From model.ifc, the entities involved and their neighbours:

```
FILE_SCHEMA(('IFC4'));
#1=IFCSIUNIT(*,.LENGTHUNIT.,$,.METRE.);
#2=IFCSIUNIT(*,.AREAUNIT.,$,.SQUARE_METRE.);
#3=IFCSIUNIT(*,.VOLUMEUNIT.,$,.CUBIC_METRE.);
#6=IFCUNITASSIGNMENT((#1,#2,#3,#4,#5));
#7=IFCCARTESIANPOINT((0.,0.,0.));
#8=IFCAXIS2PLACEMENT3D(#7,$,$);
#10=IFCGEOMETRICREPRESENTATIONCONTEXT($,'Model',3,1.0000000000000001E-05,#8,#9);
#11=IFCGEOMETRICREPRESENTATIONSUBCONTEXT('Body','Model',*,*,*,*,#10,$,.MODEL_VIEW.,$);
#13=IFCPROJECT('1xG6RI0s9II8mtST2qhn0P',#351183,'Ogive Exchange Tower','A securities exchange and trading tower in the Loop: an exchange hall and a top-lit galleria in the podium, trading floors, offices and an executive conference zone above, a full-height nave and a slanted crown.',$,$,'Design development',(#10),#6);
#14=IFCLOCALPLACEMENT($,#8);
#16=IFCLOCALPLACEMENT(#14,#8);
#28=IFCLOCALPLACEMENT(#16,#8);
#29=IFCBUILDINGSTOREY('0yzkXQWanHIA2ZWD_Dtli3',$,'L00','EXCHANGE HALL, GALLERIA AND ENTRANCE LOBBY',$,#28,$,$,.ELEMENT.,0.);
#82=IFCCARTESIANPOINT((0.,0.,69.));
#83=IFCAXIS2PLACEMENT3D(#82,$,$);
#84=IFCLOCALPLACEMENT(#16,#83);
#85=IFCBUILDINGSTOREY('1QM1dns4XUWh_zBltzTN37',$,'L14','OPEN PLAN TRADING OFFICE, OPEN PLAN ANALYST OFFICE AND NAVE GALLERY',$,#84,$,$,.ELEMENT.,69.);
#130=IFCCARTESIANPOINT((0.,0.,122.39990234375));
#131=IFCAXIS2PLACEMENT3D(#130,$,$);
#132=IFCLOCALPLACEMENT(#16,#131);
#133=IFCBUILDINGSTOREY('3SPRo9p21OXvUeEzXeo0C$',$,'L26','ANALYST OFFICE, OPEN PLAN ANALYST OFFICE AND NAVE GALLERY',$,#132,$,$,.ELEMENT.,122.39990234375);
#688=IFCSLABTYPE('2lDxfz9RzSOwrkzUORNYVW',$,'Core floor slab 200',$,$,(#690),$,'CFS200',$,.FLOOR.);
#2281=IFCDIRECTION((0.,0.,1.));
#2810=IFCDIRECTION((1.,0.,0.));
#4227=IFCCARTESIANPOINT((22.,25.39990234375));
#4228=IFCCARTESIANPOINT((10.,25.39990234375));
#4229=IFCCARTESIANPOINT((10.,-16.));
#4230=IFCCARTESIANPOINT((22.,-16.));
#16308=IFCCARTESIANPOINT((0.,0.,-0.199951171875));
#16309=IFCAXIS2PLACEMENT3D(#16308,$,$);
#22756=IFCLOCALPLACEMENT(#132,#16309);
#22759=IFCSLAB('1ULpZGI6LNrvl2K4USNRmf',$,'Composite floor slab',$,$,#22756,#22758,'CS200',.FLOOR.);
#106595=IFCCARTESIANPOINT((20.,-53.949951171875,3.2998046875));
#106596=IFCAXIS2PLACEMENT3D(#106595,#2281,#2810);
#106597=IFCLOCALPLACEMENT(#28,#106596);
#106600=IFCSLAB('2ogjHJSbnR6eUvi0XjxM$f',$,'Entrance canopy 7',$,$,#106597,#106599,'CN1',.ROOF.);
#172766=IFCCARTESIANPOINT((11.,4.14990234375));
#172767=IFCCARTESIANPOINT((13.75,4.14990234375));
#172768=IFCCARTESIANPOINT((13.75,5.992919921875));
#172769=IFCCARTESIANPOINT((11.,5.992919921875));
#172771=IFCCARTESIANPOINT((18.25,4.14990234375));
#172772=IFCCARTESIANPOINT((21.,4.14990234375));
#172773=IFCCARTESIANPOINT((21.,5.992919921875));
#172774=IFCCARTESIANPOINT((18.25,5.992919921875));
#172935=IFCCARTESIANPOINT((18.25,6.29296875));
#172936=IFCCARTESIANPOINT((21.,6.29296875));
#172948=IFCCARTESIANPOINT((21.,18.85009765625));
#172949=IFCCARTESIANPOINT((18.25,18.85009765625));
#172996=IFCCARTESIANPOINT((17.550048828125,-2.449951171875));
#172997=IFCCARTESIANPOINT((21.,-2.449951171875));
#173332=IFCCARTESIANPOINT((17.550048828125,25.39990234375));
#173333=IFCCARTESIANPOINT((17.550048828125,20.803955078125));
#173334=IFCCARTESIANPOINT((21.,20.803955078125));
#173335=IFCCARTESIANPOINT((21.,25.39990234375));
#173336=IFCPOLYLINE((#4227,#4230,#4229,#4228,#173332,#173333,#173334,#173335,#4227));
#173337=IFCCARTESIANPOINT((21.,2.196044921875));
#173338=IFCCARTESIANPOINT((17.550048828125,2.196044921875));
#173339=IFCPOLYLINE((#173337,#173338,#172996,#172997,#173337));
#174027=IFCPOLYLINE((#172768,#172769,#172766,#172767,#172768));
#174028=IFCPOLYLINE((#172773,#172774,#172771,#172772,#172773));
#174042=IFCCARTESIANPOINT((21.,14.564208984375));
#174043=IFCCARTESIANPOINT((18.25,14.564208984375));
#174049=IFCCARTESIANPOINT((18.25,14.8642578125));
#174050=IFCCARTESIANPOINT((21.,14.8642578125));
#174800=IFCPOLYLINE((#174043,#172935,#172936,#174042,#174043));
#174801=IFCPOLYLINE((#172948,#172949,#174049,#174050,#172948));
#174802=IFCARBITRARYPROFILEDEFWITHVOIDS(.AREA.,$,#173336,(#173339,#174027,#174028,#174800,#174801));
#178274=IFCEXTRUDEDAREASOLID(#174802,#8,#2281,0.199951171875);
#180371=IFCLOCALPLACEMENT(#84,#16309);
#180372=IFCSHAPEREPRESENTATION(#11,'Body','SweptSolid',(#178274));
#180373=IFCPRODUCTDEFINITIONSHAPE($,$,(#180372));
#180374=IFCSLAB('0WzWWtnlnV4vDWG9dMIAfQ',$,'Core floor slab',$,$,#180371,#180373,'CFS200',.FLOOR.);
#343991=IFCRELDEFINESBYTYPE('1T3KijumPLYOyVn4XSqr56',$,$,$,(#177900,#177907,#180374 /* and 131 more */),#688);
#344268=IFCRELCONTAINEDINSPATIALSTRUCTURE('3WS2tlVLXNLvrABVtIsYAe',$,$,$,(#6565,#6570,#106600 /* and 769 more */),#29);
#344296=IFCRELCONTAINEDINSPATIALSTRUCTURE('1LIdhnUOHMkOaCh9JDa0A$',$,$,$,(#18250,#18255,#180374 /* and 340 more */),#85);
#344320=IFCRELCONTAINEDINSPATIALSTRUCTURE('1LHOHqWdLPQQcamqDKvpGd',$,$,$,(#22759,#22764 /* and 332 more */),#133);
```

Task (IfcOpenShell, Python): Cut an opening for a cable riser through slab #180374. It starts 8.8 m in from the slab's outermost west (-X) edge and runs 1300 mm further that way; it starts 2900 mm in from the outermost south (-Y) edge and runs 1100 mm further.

```python
import numpy as np
import ifcopenshell
import ifcopenshell.api.feature
import ifcopenshell.api.geometry
import ifcopenshell.api.root
import ifcopenshell.geom
import ifcopenshell.util.placement
import ifcopenshell.util.representation
import ifcopenshell.util.shape
import ifcopenshell.util.unit

model = ifcopenshell.open("model.ifc")
unit_scale = ifcopenshell.util.unit.calculate_unit_scale(model)
settings = ifcopenshell.geom.settings()


def volume(element):
    """Net volume in cubic metres, openings subtracted."""
    shape = ifcopenshell.geom.create_shape(settings, element)
    return ifcopenshell.util.shape.get_volume(shape.geometry)


slab = model.by_guid("0WzWWtnlnV4vDWG9dMIAfQ")
before = volume(slab)

# Extent in the slab's own axes, in metres. The edges named are its -X and -Y sides.
slab_shape = ifcopenshell.geom.create_shape(settings, slab)
vertices = ifcopenshell.util.shape.get_vertices(slab_shape.geometry)
x_min, y_min, bottom = vertices.min(axis=0)
top = vertices[:, 2].max()

opening = ifcopenshell.api.root.create_entity(model, ifc_class="IfcOpeningElement", name="Cable riser opening", predefined_type="OPENING")
context = ifcopenshell.util.representation.get_context(model, "Model", "Body", "MODEL_VIEW")
width, depth = 1.3, 1.1
outline = [(0.0, 0.0), (width, 0.0), (width, depth), (0.0, depth), (0.0, 0.0)]
# Overshoot both faces by 50 mm so the cut is clean.
shape = ifcopenshell.api.geometry.add_slab_representation(
    model, context=context, depth=top - bottom + 0.1, polyline=outline
)
ifcopenshell.api.geometry.assign_representation(model, product=opening, representation=shape)

matrix = ifcopenshell.util.placement.get_local_placement(slab.ObjectPlacement)
matrix[:, 3] = matrix @ np.append(np.array([x_min + 8.8, y_min + 2.9, bottom - 0.05]) / unit_scale, 1.0)
ifcopenshell.api.geometry.edit_object_placement(model, product=opening, matrix=matrix, is_si=False)
ifcopenshell.api.feature.add_feature(model, feature=opening, element=slab)

after = volume(slab)

print(f"slab volume {before:.3f} -> {after:.3f} m3")

model.write("model_v2.ifc")
```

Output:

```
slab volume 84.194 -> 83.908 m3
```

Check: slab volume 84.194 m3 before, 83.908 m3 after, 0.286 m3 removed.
